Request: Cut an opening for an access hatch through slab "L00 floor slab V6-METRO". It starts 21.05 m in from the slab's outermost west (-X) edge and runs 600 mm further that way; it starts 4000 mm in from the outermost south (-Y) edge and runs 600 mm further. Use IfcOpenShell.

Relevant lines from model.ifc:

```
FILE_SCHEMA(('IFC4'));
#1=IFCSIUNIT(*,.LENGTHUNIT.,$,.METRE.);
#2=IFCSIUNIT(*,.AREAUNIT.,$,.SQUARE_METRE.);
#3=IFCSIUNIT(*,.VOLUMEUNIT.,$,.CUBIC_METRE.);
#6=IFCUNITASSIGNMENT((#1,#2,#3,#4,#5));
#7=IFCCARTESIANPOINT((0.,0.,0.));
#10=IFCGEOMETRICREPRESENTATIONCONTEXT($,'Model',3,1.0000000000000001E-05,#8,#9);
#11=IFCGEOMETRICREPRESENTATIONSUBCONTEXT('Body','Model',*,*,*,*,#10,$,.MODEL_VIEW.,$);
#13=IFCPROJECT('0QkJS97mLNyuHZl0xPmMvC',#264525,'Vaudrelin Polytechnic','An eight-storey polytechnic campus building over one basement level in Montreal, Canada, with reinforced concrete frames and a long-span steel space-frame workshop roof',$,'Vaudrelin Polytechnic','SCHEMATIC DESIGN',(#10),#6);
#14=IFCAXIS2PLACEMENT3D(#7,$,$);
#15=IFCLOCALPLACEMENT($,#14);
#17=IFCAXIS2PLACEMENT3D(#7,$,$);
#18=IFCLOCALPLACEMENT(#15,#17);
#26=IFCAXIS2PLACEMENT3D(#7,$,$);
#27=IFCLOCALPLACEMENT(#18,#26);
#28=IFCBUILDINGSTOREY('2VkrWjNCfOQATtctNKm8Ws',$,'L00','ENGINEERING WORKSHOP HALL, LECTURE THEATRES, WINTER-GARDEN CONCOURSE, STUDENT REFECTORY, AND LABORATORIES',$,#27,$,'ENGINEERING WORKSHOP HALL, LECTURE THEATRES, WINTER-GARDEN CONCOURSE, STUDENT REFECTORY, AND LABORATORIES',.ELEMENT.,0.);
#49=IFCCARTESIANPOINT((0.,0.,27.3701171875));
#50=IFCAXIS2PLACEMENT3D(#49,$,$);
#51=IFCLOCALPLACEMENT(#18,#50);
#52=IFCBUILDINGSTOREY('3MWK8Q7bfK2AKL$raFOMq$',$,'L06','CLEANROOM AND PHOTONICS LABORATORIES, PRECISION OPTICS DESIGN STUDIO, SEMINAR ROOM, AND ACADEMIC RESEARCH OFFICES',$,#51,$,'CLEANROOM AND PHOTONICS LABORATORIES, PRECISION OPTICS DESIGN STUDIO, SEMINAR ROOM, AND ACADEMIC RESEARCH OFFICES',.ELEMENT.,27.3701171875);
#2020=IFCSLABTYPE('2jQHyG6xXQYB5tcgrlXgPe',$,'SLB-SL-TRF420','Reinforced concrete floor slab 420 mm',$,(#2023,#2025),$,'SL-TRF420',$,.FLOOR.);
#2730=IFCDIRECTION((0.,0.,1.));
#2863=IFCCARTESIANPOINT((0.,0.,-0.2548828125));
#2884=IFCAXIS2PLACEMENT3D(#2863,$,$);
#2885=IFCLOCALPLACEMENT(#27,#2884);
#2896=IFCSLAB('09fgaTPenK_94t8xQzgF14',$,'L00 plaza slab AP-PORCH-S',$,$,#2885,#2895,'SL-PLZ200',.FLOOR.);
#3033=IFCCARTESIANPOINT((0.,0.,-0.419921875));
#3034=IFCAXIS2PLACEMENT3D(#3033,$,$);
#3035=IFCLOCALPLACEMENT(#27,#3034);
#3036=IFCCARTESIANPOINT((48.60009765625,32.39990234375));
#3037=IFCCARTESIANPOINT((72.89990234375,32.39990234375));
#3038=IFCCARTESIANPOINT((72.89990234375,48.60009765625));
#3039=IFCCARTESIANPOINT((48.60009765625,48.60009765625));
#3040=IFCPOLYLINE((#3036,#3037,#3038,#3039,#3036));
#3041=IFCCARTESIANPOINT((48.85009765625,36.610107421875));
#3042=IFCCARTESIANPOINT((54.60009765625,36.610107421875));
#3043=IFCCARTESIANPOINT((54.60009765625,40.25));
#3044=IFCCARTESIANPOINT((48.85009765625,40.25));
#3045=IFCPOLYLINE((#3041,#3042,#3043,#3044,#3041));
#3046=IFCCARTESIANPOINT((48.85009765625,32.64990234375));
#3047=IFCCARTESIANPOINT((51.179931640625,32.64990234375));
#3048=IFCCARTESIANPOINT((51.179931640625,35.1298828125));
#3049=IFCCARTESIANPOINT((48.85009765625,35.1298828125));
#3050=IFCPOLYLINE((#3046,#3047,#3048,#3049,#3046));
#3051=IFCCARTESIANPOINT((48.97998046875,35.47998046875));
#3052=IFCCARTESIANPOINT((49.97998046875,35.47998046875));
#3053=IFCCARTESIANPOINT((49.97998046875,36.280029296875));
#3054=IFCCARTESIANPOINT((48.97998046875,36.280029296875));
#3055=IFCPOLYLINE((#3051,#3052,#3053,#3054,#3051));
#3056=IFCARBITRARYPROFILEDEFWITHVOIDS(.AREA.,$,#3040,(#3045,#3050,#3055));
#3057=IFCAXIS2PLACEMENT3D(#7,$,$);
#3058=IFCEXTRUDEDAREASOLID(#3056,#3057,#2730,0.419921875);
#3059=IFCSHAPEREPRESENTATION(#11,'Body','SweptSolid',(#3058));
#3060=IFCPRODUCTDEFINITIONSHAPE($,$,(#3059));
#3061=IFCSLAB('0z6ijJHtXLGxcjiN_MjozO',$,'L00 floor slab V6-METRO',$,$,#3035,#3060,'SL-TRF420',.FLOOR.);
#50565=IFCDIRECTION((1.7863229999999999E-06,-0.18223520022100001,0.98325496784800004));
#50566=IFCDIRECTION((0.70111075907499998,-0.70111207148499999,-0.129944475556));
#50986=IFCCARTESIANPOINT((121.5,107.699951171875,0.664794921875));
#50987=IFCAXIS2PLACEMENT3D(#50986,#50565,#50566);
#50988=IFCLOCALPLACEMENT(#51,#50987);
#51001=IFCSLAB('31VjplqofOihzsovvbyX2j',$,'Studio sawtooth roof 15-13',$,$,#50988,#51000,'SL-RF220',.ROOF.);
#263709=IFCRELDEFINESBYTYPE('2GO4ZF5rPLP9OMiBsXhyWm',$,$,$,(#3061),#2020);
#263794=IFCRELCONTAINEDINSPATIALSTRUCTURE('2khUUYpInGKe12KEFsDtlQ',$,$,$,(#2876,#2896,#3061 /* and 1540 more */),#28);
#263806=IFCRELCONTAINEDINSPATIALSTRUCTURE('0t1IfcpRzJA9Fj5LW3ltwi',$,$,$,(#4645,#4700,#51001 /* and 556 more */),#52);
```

```python
import numpy as np
import ifcopenshell
import ifcopenshell.api.feature
import ifcopenshell.api.geometry
import ifcopenshell.api.root
import ifcopenshell.geom
import ifcopenshell.util.placement
import ifcopenshell.util.representation
import ifcopenshell.util.shape
import ifcopenshell.util.unit

model = ifcopenshell.open("model.ifc")
unit_scale = ifcopenshell.util.unit.calculate_unit_scale(model)
settings = ifcopenshell.geom.settings()


def volume(element):
    """Net volume in cubic metres, openings subtracted."""
    shape = ifcopenshell.geom.create_shape(settings, element)
    return ifcopenshell.util.shape.get_volume(shape.geometry)


slab = model.by_guid("0z6ijJHtXLGxcjiN_MjozO")
before = volume(slab)

# Extent in the slab's own axes, in metres. The edges named are its -X and -Y sides.
slab_shape = ifcopenshell.geom.create_shape(settings, slab)
vertices = ifcopenshell.util.shape.get_vertices(slab_shape.geometry)
x_min, y_min, bottom = vertices.min(axis=0)
top = vertices[:, 2].max()

opening = ifcopenshell.api.root.create_entity(model, ifc_class="IfcOpeningElement", name="Access hatch opening", predefined_type="OPENING")
context = ifcopenshell.util.representation.get_context(model, "Model", "Body", "MODEL_VIEW")
width, depth = 0.6, 0.6
outline = [(0.0, 0.0), (width, 0.0), (width, depth), (0.0, depth), (0.0, 0.0)]
# Overshoot both faces by 50 mm so the cut is clean.
shape = ifcopenshell.api.geometry.add_slab_representation(
    model, context=context, depth=top - bottom + 0.1, polyline=outline
)
ifcopenshell.api.geometry.assign_representation(model, product=opening, representation=shape)

matrix = ifcopenshell.util.placement.get_local_placement(slab.ObjectPlacement)
matrix[:, 3] = matrix @ np.append(np.array([x_min + 21.05, y_min + 4, bottom - 0.05]) / unit_scale, 1.0)
ifcopenshell.api.geometry.edit_object_placement(model, product=opening, matrix=matrix, is_si=False)
ifcopenshell.api.feature.add_feature(model, feature=opening, element=slab)

after = volume(slab)

print(f"slab volume {before:.3f} -> {after:.3f} m3")

model.write("model_rev.ifc")
```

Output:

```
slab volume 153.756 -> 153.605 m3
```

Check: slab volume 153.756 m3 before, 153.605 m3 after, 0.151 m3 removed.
